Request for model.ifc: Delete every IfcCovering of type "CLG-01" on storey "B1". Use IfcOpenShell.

First a look at what the model holds.

```python
import ifcopenshell
import ifcopenshell.util.element

model = ifcopenshell.open("model.ifc")
print(model.schema)
storey = next(s for s in model.by_type("IfcBuildingStorey") if s.Name == "B1")
coverings = [e for e in ifcopenshell.util.element.get_decomposition(storey) if e.is_a("IfcCovering")]
seen = {}
for e in coverings:
    element_type = ifcopenshell.util.element.get_type(e)
    name = element_type.Name if element_type not in (None, e) else None
    seen[name] = seen.get(name, 0) + 1
for name, count in sorted(seen.items(), key=str):
    print(count, "x", name)
```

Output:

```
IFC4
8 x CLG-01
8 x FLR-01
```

```python
import ifcopenshell
import ifcopenshell.api.root
import ifcopenshell.util.element

model = ifcopenshell.open("model.ifc")

storey = next(s for s in model.by_type("IfcBuildingStorey") if s.Name == "B1")
coverings = [e for e in ifcopenshell.util.element.get_decomposition(storey) if e.is_a("IfcCovering")]
targets = [e for e in coverings if (t := ifcopenshell.util.element.get_type(e)) not in (None, e) and t.Name == "CLG-01"]

for e in targets:
    ifcopenshell.api.root.remove_product(model, product=e)
print(len(targets), "removed")

model.write("model_updated.ifc")
```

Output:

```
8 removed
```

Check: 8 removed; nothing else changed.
